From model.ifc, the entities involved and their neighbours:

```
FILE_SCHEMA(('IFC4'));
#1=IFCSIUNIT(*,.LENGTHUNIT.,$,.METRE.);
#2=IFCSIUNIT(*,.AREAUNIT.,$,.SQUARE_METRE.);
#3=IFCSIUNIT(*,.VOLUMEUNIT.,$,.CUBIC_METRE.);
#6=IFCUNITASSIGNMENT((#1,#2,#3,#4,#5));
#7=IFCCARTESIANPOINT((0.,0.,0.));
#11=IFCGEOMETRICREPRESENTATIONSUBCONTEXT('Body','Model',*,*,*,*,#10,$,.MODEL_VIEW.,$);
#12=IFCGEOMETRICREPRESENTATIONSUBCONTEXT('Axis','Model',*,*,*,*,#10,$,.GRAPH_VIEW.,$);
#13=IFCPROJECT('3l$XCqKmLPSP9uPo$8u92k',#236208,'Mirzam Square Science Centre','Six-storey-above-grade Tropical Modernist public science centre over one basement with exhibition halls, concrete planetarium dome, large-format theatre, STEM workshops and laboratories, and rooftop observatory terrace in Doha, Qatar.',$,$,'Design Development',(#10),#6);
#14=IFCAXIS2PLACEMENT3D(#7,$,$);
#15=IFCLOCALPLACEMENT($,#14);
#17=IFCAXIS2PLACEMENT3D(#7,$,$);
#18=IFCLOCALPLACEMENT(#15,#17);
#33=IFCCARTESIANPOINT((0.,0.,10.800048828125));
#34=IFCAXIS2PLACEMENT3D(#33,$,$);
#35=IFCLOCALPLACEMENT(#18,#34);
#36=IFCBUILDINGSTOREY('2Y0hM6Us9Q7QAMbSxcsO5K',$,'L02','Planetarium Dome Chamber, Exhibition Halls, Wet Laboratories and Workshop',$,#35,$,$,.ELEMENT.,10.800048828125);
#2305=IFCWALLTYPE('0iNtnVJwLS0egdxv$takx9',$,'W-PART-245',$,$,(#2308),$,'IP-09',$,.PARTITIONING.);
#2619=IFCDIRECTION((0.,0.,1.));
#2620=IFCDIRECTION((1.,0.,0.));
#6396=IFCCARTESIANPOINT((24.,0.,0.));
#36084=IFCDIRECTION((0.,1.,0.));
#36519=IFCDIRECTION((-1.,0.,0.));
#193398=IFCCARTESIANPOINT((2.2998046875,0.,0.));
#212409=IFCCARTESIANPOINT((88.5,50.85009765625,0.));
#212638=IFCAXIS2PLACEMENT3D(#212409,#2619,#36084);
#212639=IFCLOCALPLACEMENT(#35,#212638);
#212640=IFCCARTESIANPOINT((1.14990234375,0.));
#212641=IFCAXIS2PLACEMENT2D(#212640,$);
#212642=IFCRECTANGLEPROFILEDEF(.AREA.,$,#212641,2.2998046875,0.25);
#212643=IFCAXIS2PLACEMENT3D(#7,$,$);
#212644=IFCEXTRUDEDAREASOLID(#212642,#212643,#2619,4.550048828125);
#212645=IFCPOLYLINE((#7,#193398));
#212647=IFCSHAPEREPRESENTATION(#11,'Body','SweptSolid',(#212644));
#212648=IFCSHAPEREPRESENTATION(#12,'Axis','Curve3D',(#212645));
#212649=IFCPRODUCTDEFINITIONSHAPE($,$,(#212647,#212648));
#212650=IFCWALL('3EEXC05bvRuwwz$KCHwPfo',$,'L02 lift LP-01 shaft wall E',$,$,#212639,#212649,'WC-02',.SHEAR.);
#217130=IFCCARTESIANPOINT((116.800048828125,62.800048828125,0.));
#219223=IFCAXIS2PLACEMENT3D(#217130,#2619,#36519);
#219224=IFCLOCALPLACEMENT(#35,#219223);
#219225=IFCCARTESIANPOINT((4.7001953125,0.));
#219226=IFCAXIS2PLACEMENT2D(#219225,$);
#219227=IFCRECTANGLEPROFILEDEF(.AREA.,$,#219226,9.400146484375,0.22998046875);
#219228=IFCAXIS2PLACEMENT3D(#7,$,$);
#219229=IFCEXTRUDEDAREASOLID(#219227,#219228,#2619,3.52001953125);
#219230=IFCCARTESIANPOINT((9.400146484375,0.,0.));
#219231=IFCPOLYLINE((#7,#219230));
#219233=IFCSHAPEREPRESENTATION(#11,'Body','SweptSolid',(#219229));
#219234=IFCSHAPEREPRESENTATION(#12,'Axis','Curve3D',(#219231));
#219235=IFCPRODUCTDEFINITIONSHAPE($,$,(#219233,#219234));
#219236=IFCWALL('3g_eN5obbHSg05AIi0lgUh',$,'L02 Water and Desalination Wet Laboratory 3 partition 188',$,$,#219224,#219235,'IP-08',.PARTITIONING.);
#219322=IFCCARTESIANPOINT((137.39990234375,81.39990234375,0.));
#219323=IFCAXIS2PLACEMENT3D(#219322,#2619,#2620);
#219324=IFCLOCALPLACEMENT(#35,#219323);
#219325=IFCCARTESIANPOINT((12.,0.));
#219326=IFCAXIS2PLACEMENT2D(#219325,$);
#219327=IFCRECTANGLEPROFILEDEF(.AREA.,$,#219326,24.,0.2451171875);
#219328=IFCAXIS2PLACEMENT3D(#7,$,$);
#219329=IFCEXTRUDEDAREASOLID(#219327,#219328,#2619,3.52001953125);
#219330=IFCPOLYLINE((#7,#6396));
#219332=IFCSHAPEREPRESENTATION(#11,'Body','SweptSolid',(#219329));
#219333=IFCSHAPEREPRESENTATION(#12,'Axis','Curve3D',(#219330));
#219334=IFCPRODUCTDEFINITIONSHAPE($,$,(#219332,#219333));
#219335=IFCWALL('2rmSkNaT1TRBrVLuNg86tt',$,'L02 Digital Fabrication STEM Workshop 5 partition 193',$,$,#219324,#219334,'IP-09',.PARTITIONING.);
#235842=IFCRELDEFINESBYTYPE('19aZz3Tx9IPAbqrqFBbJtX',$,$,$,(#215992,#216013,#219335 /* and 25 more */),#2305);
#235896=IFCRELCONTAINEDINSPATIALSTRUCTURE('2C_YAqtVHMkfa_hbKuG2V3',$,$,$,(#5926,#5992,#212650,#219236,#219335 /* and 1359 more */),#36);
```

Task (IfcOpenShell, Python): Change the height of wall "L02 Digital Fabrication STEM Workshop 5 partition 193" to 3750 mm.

```python
import ifcopenshell
import ifcopenshell.geom
import ifcopenshell.util.representation
import ifcopenshell.util.shape

model = ifcopenshell.open("model.ifc")
settings = ifcopenshell.geom.settings()


def volume(element):
    """Net volume in cubic metres, openings subtracted."""
    shape = ifcopenshell.geom.create_shape(settings, element)
    return ifcopenshell.util.shape.get_volume(shape.geometry)


wall = model.by_guid("2rmSkNaT1TRBrVLuNg86tt")
before = volume(wall)

body = ifcopenshell.util.representation.get_representation(wall, "Model", "Body")
solid = body.Items[0]
old_height = solid.Depth
solid.Depth = 3.75
after = volume(wall)

print(f"height {old_height:g} -> {solid.Depth:g}, volume {before:.3f} -> {after:.3f} m3")

model.write("model_updated.ifc")
```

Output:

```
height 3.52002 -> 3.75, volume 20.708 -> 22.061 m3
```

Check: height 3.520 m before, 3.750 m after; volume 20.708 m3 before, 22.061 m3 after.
